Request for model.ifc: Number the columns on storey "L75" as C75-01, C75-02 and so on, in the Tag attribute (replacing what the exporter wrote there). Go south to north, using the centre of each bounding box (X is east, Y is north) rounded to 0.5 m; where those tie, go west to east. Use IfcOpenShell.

First a look at what the model holds.

```python
import ifcopenshell
import ifcopenshell.util.element
import ifcopenshell.util.placement

model = ifcopenshell.open("model.ifc")
print(model.schema)
storey = next(s for s in model.by_type("IfcBuildingStorey") if s.Name == "L75")
columns = [e for e in ifcopenshell.util.element.get_decomposition(storey) if e.is_a("IfcColumn")]
for e in sorted(columns, key=lambda e: e.id()):
    origin = ifcopenshell.util.placement.get_local_placement(e.ObjectPlacement)[:3, 3]
    print(e.id(), e.Tag, e.Name, origin.round(2) + 0.0, sep=" | ")
```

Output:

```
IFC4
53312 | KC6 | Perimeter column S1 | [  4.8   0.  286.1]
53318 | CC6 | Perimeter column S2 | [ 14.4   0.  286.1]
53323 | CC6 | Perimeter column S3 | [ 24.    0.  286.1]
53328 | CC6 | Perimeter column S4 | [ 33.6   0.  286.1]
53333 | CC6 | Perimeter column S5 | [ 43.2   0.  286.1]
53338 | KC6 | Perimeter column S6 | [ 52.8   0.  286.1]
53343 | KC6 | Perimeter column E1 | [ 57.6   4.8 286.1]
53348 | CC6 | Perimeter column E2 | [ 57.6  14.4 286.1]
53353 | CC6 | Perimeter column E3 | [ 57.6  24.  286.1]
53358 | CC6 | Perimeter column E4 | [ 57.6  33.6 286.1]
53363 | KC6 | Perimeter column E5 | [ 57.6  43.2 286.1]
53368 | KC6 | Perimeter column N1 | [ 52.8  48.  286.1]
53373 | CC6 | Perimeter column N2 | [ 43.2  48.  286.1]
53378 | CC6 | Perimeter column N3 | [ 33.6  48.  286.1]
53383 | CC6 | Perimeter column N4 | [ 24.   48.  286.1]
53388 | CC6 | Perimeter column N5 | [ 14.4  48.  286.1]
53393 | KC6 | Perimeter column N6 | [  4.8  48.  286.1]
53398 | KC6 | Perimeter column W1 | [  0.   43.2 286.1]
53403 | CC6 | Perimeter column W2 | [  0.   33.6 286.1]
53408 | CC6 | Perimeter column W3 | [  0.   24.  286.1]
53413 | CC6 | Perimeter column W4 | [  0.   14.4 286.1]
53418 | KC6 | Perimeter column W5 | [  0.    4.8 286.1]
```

```python
import ifcopenshell
import ifcopenshell.geom
import ifcopenshell.util.element
import ifcopenshell.util.shape

model = ifcopenshell.open("model.ifc")
settings = ifcopenshell.geom.settings()
settings.set("use-world-coords", True)


def centre(element):
    shape = ifcopenshell.geom.create_shape(settings, element)
    return ifcopenshell.util.shape.get_bbox_centroid(shape.geometry)


storey = next(s for s in model.by_type("IfcBuildingStorey") if s.Name == "L75")
columns = [e for e in ifcopenshell.util.element.get_decomposition(storey) if e.is_a("IfcColumn")]

# Insertion points can sit at a corner or the storey origin, so sort by the geometry (in metres).
centres = {e: centre(e) for e in columns}
columns.sort(key=lambda e: (round(centres[e][1] / 0.5), centres[e][0]))

for i, e in enumerate(columns, start=1):
    number = f"C75-{i:02d}"
    e.Tag = number
    print(e.id(), number)

model.write("model_updated.ifc")
```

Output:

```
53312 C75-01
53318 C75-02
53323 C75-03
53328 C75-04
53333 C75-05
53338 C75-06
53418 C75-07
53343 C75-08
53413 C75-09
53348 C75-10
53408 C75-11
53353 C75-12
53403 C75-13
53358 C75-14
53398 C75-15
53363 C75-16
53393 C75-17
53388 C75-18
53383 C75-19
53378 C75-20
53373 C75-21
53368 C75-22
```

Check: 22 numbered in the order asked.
